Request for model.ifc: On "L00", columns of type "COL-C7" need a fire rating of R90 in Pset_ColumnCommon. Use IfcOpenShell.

First a look at what the model holds.

```python
import ifcopenshell
import ifcopenshell.util.element

model = ifcopenshell.open("model.ifc")
print(model.schema)
storey = next(s for s in model.by_type("IfcBuildingStorey") if s.Name == "L00")
columns = [e for e in ifcopenshell.util.element.get_decomposition(storey) if e.is_a("IfcColumn")]
seen = {}
for e in columns:
    element_type = ifcopenshell.util.element.get_type(e)
    key = (element_type.Name if element_type != e and element_type else None, ifcopenshell.util.element.get_pset(e, "Pset_ColumnCommon", "FireRating"))
    seen[key] = seen.get(key, 0) + 1
for (name, value), count in sorted(seen.items(), key=str):
    print(count, "x", name, "|", value)
```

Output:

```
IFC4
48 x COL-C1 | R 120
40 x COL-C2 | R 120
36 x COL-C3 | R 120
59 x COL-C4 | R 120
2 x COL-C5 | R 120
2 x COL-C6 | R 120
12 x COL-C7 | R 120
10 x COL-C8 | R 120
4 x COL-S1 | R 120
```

```python
import ifcopenshell
import ifcopenshell.api.pset
import ifcopenshell.util.element

model = ifcopenshell.open("model.ifc")

storey = next(s for s in model.by_type("IfcBuildingStorey") if s.Name == "L00")
columns = [e for e in ifcopenshell.util.element.get_decomposition(storey) if e.is_a("IfcColumn")]

count = 0
for e in columns:
    element_type = ifcopenshell.util.element.get_type(e)
    if element_type in (None, e) or element_type.Name != "COL-C7":
        continue
    # add_pset returns the element's existing set when there is one.
    pset = ifcopenshell.api.pset.add_pset(model, product=e, name="Pset_ColumnCommon")
    ifcopenshell.api.pset.edit_pset(model, pset=pset, properties={"FireRating": "R90"})
    count += 1

print(count, "columns updated")

model.write("model_updated.ifc")
```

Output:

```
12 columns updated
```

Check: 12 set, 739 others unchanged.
